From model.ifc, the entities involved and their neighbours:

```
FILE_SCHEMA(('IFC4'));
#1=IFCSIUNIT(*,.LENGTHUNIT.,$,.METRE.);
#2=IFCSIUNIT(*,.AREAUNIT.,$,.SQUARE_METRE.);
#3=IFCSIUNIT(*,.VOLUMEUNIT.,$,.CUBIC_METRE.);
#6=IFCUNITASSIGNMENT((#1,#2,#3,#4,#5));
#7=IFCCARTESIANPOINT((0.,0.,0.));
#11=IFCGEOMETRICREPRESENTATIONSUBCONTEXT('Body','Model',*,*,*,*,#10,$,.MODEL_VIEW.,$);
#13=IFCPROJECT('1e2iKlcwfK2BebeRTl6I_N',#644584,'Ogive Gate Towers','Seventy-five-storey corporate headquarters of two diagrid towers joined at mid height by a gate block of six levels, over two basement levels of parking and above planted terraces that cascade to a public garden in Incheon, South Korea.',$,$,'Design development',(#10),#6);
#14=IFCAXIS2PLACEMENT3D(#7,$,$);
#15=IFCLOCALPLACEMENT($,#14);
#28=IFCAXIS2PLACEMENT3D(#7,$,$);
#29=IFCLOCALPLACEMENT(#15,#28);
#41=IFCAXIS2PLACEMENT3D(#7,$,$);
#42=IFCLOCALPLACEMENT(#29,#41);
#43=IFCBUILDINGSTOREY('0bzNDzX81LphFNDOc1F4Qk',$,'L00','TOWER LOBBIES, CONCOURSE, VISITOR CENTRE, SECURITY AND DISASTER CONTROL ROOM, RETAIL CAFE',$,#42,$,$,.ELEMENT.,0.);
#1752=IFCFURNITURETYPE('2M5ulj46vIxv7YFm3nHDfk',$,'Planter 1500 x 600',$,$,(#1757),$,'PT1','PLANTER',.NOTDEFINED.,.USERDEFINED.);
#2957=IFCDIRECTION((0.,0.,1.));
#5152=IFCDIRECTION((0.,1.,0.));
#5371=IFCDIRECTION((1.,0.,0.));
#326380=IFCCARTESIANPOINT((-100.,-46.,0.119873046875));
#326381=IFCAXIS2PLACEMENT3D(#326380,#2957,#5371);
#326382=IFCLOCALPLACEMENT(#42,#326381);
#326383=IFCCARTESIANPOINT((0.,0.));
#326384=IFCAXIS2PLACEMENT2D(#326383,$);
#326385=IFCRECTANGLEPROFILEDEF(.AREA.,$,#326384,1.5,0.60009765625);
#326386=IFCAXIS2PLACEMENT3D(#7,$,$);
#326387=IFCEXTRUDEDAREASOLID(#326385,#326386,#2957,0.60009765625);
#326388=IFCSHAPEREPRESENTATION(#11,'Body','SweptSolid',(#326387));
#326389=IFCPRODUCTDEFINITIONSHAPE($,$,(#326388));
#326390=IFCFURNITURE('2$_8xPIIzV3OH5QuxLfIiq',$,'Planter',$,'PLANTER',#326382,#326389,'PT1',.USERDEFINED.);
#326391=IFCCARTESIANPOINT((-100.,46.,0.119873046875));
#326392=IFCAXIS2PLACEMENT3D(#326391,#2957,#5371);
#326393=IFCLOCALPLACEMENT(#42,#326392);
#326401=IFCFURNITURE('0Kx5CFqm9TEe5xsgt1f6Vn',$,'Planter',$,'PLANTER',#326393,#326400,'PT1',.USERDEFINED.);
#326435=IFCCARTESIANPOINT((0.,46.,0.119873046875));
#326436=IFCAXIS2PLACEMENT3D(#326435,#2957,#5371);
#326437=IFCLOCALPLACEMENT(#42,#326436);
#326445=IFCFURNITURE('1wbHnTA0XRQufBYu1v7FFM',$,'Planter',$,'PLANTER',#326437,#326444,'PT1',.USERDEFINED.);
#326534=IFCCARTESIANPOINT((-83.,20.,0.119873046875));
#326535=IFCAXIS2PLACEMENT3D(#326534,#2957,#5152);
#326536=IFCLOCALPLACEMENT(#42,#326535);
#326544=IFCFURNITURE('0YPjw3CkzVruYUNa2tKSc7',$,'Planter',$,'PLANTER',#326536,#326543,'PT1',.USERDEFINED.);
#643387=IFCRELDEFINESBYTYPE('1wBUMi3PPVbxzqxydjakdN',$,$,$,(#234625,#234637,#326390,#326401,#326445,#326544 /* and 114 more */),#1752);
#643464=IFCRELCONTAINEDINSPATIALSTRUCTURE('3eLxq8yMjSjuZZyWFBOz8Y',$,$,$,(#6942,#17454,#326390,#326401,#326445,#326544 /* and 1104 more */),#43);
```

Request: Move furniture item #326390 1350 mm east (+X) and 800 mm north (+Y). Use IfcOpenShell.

```python
import ifcopenshell
import ifcopenshell.api.geometry
import ifcopenshell.util.placement
import ifcopenshell.util.unit

model = ifcopenshell.open("model.ifc")
unit_scale = ifcopenshell.util.unit.calculate_unit_scale(model)

item = model.by_guid("2$_8xPIIzV3OH5QuxLfIiq")
matrix = ifcopenshell.util.placement.get_local_placement(item.ObjectPlacement)
matrix[0, 3] += 1.35 / unit_scale
matrix[1, 3] += 0.8 / unit_scale
ifcopenshell.api.geometry.edit_object_placement(model, product=item, matrix=matrix, is_si=False)

print(ifcopenshell.util.placement.get_local_placement(item.ObjectPlacement).round(3) + 0.0)

model.write("model_v2.ifc")
```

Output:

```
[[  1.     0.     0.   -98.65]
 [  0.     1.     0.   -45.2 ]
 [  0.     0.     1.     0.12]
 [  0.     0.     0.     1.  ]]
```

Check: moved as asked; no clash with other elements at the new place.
